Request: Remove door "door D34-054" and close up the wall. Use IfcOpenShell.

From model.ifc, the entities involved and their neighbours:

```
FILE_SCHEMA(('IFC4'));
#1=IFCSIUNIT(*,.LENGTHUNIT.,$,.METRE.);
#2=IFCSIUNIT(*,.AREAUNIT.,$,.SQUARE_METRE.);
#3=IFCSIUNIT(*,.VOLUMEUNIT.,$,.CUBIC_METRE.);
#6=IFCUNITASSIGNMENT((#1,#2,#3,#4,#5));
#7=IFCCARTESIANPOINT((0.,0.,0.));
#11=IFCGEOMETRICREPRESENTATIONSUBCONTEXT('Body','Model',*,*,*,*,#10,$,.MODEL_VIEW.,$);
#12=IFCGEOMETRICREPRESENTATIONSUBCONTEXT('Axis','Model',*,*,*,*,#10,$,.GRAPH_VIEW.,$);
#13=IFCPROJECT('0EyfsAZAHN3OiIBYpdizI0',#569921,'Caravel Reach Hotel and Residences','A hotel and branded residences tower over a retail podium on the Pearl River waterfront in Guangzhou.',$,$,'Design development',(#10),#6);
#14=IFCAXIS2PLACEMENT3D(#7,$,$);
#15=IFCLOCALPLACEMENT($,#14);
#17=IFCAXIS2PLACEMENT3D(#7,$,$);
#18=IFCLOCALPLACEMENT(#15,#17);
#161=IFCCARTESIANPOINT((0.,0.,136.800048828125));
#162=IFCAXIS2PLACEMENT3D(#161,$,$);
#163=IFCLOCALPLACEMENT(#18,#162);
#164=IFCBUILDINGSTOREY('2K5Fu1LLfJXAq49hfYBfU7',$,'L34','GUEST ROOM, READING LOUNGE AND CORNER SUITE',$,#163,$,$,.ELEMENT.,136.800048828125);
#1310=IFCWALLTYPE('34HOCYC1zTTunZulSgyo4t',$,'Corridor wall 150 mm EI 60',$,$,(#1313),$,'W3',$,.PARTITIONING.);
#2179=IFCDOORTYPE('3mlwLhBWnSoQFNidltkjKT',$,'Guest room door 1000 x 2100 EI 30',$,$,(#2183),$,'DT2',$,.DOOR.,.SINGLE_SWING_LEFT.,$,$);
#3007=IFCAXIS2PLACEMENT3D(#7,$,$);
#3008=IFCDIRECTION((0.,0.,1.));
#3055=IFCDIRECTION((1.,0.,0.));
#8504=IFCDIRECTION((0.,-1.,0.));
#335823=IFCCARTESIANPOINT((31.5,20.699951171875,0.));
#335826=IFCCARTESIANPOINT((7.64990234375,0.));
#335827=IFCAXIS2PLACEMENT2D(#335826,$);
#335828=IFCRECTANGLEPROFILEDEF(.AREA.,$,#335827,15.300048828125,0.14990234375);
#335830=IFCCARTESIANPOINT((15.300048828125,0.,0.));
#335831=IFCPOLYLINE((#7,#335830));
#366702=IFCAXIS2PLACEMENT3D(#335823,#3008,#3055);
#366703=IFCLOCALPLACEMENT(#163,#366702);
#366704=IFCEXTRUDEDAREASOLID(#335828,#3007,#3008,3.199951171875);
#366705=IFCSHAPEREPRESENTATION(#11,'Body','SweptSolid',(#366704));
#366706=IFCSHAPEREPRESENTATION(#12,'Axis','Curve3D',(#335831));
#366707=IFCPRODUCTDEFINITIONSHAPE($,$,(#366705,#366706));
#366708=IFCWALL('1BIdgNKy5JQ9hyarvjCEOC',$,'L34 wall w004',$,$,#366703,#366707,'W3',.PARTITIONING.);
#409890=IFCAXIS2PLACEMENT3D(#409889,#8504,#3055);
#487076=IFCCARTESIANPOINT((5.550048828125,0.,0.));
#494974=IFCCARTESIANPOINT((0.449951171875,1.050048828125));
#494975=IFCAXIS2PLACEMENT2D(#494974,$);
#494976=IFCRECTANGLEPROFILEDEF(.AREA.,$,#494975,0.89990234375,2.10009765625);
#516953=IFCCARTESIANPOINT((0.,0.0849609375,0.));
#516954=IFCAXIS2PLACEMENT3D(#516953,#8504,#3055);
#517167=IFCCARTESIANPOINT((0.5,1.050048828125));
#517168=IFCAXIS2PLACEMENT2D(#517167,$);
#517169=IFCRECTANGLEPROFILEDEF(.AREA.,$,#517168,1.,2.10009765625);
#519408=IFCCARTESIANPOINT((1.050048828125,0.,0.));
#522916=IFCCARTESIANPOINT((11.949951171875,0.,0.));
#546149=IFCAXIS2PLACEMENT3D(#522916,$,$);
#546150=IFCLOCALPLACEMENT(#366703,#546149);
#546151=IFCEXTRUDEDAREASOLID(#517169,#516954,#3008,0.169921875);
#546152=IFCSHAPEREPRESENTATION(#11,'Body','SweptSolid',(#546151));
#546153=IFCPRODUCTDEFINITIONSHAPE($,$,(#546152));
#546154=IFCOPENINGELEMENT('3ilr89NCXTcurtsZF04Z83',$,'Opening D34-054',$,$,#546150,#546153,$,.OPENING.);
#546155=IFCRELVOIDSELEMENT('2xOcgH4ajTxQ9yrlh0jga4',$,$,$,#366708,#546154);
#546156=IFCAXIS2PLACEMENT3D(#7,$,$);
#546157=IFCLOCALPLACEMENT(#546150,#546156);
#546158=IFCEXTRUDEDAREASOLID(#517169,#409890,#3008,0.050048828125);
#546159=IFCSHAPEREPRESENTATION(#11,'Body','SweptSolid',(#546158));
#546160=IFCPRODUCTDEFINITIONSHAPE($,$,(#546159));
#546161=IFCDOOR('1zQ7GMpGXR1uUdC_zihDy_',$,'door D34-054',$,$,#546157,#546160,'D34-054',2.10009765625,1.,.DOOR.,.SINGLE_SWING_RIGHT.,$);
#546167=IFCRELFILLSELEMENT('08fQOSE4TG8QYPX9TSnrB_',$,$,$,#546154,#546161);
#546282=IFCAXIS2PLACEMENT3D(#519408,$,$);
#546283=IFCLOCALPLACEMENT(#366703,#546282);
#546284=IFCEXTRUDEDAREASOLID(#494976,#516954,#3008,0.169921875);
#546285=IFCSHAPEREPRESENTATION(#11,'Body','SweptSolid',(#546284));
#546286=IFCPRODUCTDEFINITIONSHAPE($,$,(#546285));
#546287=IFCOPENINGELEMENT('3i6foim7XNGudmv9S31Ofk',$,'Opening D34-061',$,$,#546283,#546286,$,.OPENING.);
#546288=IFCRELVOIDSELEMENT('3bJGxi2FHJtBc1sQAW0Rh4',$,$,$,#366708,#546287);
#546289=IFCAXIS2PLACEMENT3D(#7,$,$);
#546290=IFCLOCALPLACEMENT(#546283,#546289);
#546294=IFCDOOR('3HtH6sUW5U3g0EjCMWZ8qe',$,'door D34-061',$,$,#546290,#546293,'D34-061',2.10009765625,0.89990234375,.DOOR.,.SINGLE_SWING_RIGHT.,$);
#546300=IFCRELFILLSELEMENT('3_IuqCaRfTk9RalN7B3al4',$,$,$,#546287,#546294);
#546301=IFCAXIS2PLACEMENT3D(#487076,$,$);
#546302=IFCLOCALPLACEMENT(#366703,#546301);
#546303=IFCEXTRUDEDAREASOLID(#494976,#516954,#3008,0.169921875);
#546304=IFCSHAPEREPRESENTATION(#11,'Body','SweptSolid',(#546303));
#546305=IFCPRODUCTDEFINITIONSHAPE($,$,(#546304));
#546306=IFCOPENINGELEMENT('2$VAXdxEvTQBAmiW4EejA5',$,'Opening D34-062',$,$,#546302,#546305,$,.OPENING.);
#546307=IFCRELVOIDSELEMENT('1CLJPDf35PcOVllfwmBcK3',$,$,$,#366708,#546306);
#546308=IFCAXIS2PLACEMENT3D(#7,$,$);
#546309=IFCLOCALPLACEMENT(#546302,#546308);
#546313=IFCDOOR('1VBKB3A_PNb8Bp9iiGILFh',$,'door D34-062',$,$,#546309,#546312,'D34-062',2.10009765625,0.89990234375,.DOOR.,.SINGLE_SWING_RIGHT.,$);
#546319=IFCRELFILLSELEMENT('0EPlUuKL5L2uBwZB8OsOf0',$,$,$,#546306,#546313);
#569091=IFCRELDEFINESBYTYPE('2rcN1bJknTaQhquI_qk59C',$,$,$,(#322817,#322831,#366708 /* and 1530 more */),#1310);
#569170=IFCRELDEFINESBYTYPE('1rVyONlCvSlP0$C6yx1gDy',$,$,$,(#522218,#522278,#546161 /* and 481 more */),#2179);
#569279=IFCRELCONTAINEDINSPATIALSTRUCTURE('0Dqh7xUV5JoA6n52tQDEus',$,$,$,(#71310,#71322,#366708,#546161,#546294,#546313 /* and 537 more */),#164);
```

```python
import ifcopenshell
import ifcopenshell.api.feature
import ifcopenshell.api.root
import ifcopenshell.geom
import ifcopenshell.util.shape

model = ifcopenshell.open("model.ifc")
settings = ifcopenshell.geom.settings()


def volume(element):
    """Net volume in cubic metres, openings subtracted."""
    shape = ifcopenshell.geom.create_shape(settings, element)
    return ifcopenshell.util.shape.get_volume(shape.geometry)


door = model.by_id(546161)
opening = door.FillsVoids[0].RelatingOpeningElement
wall = opening.VoidsElements[0].RelatingBuildingElement
before = volume(wall)

ifcopenshell.api.root.remove_product(model, product=door)
ifcopenshell.api.feature.remove_feature(model, feature=opening)

after = volume(wall)

print(f"wall volume {before:.3f} -> {after:.3f} m3")

model.write("model_v2.ifc")
```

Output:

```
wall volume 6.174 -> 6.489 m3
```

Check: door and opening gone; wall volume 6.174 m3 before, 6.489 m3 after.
